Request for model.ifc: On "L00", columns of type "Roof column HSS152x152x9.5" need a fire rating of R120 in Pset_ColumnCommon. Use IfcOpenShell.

First a look at what the model holds.

```python
import ifcopenshell
import ifcopenshell.util.element

model = ifcopenshell.open("model.ifc")
print(model.schema)
storey = next(s for s in model.by_type("IfcBuildingStorey") if s.Name == "L00")
columns = [e for e in ifcopenshell.util.element.get_decomposition(storey) if e.is_a("IfcColumn")]
seen = {}
for e in columns:
    element_type = ifcopenshell.util.element.get_type(e)
    key = (element_type.Name if element_type != e and element_type else None, ifcopenshell.util.element.get_pset(e, "Pset_ColumnCommon", "FireRating"))
    seen[key] = seen.get(key, 0) + 1
for (name, value), count in sorted(seen.items(), key=str):
    print(count, "x", name, "|", value)
```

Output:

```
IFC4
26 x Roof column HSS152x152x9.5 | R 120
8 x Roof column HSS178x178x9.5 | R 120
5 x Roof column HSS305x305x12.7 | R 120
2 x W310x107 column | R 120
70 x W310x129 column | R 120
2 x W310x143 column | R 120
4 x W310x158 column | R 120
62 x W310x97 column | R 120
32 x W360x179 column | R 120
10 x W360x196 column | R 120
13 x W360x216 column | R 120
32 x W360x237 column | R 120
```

```python
import ifcopenshell
import ifcopenshell.api.pset
import ifcopenshell.util.element

model = ifcopenshell.open("model.ifc")

storey = next(s for s in model.by_type("IfcBuildingStorey") if s.Name == "L00")
columns = [e for e in ifcopenshell.util.element.get_decomposition(storey) if e.is_a("IfcColumn")]

count = 0
for e in columns:
    element_type = ifcopenshell.util.element.get_type(e)
    if element_type in (None, e) or element_type.Name != "Roof column HSS152x152x9.5":
        continue
    # add_pset returns the element's existing set when there is one.
    pset = ifcopenshell.api.pset.add_pset(model, product=e, name="Pset_ColumnCommon")
    ifcopenshell.api.pset.edit_pset(model, pset=pset, properties={"FireRating": "R120"})
    count += 1

print(count, "columns updated")

model.write("model-out.ifc")
```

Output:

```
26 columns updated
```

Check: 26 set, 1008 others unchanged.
